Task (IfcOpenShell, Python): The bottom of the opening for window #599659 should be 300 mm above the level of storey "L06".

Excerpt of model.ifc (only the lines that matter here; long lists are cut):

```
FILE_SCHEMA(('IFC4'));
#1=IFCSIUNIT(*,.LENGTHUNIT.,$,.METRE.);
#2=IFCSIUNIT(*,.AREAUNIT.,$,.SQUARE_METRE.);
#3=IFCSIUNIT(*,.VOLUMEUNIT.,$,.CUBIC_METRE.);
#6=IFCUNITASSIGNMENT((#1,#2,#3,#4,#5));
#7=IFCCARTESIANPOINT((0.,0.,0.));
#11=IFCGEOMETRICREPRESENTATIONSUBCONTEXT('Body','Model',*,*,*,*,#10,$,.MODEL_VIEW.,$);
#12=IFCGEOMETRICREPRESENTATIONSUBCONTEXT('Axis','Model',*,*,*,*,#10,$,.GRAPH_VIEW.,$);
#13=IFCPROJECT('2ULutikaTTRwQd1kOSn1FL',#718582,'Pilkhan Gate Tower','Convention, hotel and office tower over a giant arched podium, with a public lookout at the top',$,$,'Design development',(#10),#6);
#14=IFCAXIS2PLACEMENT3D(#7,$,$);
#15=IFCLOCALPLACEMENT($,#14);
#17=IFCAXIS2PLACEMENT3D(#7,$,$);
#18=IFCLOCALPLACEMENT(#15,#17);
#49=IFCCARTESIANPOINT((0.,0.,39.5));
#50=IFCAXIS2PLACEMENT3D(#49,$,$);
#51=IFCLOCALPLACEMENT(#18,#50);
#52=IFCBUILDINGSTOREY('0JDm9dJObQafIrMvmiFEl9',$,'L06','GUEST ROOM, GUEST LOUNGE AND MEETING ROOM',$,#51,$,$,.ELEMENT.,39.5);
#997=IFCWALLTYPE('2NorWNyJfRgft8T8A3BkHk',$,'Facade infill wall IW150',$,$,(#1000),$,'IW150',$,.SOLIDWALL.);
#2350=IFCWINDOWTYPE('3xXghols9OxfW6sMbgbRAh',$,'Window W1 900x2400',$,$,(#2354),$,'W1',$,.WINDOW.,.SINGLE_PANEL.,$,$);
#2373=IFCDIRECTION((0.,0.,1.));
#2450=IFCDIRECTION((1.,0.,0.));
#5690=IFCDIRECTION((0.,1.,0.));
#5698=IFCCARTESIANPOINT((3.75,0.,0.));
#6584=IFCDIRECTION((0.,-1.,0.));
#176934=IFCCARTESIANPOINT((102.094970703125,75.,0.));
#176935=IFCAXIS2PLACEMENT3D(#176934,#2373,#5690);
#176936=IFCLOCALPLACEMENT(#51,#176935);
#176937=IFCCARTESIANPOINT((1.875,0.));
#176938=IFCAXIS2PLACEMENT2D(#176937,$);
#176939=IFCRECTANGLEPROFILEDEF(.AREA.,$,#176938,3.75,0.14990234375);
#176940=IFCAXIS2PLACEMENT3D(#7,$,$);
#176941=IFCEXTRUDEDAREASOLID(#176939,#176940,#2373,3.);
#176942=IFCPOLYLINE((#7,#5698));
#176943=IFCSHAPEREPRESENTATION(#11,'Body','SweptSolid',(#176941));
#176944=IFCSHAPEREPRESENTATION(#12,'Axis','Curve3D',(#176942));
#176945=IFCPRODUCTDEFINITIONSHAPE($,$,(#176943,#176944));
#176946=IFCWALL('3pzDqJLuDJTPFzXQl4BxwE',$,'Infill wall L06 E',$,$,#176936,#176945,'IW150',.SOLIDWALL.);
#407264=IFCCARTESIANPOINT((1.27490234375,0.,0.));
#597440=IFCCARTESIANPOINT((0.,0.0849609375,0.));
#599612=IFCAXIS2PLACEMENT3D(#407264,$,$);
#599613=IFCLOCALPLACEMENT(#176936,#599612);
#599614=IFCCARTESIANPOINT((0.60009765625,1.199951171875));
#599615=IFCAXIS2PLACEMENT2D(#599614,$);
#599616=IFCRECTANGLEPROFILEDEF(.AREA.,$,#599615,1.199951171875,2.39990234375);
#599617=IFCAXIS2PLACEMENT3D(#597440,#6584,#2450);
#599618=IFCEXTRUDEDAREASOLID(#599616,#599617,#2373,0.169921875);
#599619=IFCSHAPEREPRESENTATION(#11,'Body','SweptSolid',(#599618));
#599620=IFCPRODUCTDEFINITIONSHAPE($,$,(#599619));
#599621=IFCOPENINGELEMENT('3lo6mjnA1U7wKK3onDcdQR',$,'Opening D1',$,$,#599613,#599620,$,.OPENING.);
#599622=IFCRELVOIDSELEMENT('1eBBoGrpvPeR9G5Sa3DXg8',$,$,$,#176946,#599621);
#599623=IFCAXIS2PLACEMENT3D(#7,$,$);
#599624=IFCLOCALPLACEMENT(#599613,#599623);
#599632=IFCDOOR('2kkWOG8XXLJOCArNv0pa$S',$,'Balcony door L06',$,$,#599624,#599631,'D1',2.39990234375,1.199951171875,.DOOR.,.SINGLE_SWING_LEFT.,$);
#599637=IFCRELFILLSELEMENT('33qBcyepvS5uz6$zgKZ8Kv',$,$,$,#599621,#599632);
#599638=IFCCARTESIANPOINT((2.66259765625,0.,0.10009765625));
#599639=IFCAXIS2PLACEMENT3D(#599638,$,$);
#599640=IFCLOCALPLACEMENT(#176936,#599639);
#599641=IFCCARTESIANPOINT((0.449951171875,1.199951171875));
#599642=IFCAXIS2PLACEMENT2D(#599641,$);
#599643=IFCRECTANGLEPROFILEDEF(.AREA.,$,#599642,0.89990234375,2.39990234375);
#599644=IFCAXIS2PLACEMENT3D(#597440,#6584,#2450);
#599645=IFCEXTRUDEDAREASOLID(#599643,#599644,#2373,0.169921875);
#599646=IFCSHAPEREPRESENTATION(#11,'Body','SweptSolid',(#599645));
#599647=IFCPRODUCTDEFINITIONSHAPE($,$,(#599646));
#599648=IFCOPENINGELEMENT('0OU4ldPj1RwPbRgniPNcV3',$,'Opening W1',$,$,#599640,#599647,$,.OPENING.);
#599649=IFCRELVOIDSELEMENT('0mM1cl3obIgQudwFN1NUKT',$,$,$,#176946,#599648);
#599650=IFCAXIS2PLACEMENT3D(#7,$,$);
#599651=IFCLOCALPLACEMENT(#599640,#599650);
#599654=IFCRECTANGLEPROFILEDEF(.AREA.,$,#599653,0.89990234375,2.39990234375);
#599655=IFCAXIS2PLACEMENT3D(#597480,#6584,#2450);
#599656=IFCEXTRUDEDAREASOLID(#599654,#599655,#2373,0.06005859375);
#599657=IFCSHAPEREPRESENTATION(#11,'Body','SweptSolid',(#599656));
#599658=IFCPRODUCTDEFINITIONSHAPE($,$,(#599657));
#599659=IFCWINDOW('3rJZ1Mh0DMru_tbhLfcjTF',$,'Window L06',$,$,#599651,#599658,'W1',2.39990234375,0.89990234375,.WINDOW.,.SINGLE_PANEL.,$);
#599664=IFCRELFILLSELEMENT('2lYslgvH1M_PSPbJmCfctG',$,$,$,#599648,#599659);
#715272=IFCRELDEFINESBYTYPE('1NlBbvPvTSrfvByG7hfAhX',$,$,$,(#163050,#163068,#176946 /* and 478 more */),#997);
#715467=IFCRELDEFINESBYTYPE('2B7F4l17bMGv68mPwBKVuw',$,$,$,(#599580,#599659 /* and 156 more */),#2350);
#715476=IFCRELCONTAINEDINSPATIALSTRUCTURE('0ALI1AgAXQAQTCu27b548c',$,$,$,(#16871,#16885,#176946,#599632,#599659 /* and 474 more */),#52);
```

```python
import numpy as np
import ifcopenshell
import ifcopenshell.api.geometry
import ifcopenshell.geom
import ifcopenshell.util.element
import ifcopenshell.util.placement
import ifcopenshell.util.shape
import ifcopenshell.util.unit

model = ifcopenshell.open("model.ifc")
unit_scale = ifcopenshell.util.unit.calculate_unit_scale(model)

window = model.by_guid("3rJZ1Mh0DMru_tbhLfcjTF")
opening = window.FillsVoids[0].RelatingOpeningElement
storey = ifcopenshell.util.element.get_container(window, ifc_class="IfcBuildingStorey")
level = ifcopenshell.util.placement.get_local_placement(storey.ObjectPlacement)[2, 3]

# The opening's origin need not be at the sill, so measure its lowest point.
shape = ifcopenshell.geom.create_shape(ifcopenshell.geom.settings(), opening)
bottom = ifcopenshell.util.shape.get_shape_bottom_elevation(shape, shape.geometry) / unit_scale
dz = level + 0.3 - bottom

shift = np.array([0.0, 0.0, dz])
# The window is placed relative to its opening, so it follows when the opening moves.
matrix = ifcopenshell.util.placement.get_local_placement(opening.ObjectPlacement)
matrix[:3, 3] += shift
ifcopenshell.api.geometry.edit_object_placement(
    model, product=opening, matrix=matrix, is_si=False, should_transform_children=True
)

print(f"moved by {dz * unit_scale:+.3f} m")

model.write("model_rev.ifc")
```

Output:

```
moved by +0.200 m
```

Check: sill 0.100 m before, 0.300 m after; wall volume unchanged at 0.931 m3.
